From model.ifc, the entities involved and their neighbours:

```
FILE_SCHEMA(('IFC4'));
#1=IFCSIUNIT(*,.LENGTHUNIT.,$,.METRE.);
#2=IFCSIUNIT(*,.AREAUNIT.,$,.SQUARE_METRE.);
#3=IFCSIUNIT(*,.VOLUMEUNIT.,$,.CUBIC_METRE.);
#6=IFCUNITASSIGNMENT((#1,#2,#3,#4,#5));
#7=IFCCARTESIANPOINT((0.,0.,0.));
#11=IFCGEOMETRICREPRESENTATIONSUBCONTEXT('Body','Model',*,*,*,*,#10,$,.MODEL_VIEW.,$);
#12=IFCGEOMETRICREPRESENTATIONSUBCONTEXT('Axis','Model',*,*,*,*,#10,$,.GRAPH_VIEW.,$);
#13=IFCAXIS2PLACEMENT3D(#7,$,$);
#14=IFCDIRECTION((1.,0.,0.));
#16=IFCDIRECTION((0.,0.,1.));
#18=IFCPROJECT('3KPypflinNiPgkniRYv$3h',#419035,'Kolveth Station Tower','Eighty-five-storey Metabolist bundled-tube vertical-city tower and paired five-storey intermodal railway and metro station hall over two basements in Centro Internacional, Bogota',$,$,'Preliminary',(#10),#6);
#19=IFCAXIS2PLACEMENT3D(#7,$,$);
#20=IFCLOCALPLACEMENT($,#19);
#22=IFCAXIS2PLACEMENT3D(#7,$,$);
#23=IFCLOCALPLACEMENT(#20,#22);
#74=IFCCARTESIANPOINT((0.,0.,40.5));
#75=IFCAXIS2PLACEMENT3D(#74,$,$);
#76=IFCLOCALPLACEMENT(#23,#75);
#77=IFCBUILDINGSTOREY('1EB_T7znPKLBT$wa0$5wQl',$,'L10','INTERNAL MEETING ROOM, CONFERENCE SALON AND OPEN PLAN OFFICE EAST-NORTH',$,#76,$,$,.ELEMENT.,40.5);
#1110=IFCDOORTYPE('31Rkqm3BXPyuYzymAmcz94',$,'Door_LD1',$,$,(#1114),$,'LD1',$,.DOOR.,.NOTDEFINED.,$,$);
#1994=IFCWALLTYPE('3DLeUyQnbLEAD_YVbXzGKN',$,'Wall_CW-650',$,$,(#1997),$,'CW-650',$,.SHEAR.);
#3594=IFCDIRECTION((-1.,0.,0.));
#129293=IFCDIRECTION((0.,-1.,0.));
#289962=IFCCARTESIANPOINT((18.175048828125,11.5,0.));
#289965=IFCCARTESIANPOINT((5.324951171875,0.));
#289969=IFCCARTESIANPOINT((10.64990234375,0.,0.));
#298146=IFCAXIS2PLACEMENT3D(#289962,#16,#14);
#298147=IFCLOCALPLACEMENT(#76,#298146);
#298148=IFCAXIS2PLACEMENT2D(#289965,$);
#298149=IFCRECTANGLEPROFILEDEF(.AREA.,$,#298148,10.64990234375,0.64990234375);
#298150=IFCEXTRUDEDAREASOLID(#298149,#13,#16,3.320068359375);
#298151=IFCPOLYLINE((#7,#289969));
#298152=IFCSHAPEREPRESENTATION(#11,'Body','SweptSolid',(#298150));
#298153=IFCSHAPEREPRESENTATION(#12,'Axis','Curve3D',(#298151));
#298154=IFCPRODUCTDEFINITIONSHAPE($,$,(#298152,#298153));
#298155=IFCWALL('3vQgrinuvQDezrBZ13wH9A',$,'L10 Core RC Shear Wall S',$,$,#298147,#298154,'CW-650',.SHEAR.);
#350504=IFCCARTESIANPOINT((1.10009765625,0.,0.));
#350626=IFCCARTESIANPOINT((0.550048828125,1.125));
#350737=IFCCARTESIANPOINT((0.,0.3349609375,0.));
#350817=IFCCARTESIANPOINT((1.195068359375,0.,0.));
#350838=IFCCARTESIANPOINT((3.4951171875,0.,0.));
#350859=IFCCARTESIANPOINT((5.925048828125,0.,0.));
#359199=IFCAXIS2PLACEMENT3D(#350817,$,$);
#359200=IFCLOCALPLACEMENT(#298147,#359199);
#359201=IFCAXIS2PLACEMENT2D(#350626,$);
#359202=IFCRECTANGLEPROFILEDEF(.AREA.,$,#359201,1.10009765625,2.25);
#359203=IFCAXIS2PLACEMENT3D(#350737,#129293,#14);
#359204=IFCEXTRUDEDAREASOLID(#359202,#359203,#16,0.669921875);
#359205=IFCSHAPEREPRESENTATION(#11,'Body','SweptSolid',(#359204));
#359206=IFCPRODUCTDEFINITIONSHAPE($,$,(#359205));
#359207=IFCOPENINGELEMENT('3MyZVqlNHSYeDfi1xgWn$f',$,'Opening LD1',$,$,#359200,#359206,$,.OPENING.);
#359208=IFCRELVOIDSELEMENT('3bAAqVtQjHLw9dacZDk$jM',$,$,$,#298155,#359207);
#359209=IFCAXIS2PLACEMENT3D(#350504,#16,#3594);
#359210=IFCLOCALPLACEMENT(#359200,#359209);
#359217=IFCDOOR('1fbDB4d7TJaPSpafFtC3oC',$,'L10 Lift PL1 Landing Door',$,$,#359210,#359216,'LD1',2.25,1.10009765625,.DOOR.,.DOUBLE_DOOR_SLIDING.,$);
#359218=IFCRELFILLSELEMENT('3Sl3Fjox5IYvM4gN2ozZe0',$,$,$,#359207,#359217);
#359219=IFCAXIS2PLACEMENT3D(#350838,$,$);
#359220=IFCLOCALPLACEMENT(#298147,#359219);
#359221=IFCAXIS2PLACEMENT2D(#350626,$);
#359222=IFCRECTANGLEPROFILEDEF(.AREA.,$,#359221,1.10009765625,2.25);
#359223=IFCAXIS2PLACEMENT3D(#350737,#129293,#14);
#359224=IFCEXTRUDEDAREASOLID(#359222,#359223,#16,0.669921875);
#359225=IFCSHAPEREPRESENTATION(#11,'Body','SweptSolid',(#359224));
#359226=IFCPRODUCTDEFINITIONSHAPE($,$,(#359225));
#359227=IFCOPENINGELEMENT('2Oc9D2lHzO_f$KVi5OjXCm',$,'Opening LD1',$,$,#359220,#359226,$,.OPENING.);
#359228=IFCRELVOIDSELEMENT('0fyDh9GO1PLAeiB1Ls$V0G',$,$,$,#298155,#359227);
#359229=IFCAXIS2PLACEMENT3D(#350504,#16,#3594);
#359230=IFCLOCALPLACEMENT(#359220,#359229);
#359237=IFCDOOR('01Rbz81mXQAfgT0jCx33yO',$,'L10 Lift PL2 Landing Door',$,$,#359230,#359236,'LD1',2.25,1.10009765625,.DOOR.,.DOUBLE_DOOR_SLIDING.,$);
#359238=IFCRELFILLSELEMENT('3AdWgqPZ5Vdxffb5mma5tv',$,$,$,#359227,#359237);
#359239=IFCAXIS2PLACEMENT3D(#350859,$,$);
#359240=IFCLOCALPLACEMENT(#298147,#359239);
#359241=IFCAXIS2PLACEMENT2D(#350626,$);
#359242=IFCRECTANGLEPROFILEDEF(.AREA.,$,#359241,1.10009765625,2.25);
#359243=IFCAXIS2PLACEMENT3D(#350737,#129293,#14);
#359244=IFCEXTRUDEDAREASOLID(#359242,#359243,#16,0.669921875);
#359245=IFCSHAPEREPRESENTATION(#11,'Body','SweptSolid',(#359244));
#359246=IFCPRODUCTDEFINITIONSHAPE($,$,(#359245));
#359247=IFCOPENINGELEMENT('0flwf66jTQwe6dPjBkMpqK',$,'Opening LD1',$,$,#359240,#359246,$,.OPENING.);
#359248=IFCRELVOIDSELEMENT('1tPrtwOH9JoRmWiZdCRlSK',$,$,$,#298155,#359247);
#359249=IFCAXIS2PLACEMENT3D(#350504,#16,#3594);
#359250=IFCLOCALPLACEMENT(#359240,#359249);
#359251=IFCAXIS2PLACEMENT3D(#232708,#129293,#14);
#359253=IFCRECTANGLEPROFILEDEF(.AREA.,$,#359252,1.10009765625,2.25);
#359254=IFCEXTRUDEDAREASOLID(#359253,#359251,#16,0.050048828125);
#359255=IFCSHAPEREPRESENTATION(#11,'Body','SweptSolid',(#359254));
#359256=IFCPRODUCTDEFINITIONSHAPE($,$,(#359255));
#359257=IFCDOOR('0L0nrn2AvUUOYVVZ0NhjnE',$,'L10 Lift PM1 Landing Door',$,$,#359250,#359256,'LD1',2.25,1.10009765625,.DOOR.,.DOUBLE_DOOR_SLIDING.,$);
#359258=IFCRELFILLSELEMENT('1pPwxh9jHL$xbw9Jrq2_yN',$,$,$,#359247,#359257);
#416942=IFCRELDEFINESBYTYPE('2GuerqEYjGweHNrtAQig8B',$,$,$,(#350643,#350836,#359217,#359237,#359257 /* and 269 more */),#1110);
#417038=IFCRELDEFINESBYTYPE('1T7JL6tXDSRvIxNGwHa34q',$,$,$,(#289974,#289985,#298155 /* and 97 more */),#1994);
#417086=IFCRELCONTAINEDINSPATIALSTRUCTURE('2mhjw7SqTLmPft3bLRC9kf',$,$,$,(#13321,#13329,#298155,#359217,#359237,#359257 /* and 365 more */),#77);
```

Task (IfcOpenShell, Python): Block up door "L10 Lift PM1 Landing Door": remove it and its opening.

```python
import ifcopenshell
import ifcopenshell.api.feature
import ifcopenshell.api.root
import ifcopenshell.geom
import ifcopenshell.util.shape

model = ifcopenshell.open("model.ifc")
settings = ifcopenshell.geom.settings()


def volume(element):
    """Net volume in cubic metres, openings subtracted."""
    shape = ifcopenshell.geom.create_shape(settings, element)
    return ifcopenshell.util.shape.get_volume(shape.geometry)


door = model.by_id(359257)
opening = door.FillsVoids[0].RelatingOpeningElement
wall = opening.VoidsElements[0].RelatingBuildingElement
before = volume(wall)

ifcopenshell.api.root.remove_product(model, product=door)
ifcopenshell.api.feature.remove_feature(model, feature=opening)

after = volume(wall)

print(f"wall volume {before:.3f} -> {after:.3f} m3")

model.write("model_edited.ifc")
```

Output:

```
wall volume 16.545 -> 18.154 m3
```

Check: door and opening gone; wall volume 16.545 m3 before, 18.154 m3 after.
